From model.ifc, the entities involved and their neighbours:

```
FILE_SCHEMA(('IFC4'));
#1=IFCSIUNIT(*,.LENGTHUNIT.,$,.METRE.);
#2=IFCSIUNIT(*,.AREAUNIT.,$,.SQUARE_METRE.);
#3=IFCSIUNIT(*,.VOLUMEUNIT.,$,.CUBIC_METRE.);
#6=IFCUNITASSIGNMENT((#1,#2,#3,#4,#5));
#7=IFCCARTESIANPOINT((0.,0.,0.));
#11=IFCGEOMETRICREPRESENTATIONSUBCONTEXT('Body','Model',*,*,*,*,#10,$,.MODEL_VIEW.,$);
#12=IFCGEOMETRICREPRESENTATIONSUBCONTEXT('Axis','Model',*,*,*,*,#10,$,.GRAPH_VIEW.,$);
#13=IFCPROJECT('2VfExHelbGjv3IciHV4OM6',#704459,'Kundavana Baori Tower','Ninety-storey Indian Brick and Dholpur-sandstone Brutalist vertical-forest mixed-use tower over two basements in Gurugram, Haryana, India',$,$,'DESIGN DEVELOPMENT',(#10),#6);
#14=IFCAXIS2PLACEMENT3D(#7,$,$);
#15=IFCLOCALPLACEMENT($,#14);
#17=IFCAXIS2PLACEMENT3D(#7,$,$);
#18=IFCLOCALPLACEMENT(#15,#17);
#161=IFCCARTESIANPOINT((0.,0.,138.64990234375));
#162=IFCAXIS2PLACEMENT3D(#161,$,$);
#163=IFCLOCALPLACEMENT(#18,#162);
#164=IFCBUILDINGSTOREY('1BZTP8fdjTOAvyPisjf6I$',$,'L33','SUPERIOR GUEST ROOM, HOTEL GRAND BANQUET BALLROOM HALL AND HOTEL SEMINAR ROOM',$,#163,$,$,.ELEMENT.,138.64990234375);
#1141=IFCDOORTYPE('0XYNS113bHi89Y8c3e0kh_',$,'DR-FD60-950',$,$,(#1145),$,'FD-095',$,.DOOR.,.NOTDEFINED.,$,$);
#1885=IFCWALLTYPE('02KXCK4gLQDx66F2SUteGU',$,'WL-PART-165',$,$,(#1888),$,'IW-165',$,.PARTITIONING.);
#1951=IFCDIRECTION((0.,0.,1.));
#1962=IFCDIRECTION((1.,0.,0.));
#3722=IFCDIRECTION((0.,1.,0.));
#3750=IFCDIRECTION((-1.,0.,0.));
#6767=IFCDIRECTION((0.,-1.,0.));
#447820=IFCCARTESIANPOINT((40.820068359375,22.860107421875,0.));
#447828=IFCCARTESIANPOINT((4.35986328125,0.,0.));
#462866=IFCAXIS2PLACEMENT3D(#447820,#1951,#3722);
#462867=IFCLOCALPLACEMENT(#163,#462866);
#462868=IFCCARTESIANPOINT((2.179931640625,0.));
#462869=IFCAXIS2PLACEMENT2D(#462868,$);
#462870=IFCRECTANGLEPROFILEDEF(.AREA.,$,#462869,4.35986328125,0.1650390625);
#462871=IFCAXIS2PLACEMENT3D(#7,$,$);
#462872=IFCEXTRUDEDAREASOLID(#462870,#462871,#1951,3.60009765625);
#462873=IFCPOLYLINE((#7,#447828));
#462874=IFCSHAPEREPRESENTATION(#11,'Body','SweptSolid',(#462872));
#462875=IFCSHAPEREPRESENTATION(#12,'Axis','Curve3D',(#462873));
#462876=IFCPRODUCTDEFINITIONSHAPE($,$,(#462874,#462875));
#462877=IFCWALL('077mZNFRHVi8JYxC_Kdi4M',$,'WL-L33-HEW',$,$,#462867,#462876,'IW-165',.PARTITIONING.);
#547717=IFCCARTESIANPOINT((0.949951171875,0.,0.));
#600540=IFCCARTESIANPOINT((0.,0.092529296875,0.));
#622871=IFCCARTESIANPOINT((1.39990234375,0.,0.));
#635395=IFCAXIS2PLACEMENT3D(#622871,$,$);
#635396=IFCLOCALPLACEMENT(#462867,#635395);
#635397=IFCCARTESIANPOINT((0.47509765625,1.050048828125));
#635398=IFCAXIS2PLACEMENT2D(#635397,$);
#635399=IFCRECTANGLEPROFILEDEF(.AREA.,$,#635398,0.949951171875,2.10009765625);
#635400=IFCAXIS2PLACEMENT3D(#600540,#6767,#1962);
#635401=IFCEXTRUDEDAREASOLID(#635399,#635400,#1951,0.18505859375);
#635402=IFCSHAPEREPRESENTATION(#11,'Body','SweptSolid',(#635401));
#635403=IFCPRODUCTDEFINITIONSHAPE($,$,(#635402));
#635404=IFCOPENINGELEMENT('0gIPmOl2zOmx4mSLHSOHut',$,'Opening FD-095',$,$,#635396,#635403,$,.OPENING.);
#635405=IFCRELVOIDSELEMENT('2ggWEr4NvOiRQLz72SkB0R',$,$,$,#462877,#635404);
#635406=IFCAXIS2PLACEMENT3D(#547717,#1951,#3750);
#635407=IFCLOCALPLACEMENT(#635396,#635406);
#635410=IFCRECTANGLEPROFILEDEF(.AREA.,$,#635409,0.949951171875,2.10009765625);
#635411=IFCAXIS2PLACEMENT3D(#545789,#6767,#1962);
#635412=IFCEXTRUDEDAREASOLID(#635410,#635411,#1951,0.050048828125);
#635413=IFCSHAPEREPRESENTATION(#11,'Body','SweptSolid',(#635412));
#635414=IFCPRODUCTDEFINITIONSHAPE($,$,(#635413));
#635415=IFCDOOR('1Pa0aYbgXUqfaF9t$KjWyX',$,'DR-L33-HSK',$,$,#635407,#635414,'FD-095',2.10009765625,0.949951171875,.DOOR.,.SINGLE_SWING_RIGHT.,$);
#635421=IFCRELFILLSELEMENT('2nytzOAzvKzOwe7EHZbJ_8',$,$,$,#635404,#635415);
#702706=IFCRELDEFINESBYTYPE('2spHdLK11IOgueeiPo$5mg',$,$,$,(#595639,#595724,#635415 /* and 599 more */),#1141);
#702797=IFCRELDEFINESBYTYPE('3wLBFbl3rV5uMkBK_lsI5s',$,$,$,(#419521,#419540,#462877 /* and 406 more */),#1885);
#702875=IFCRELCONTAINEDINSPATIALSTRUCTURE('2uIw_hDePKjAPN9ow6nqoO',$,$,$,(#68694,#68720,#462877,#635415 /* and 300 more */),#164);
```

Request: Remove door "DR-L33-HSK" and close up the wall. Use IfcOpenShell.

```python
import ifcopenshell
import ifcopenshell.api.feature
import ifcopenshell.api.root
import ifcopenshell.geom
import ifcopenshell.util.shape

model = ifcopenshell.open("model.ifc")
settings = ifcopenshell.geom.settings()


def volume(element):
    """Net volume in cubic metres, openings subtracted."""
    shape = ifcopenshell.geom.create_shape(settings, element)
    return ifcopenshell.util.shape.get_volume(shape.geometry)


door = model.by_guid("1Pa0aYbgXUqfaF9t$KjWyX")
opening = door.FillsVoids[0].RelatingOpeningElement
wall = opening.VoidsElements[0].RelatingBuildingElement
before = volume(wall)

ifcopenshell.api.root.remove_product(model, product=door)
ifcopenshell.api.feature.remove_feature(model, feature=opening)

after = volume(wall)

print(f"wall volume {before:.3f} -> {after:.3f} m3")

model.write("model_rev.ifc")
```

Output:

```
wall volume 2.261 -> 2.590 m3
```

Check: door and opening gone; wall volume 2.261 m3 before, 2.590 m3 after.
